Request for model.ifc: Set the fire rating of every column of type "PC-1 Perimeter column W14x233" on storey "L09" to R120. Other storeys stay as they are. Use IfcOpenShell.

First a look at what the model holds.

```python
import ifcopenshell
import ifcopenshell.util.element

model = ifcopenshell.open("model.ifc")
print(model.schema)
storey = next(s for s in model.by_type("IfcBuildingStorey") if s.Name == "L09")
columns = [e for e in ifcopenshell.util.element.get_decomposition(storey) if e.is_a("IfcColumn")]
seen = {}
for e in columns:
    element_type = ifcopenshell.util.element.get_type(e)
    key = (element_type.Name if element_type != e and element_type else None, ifcopenshell.util.element.get_pset(e, "Pset_ColumnCommon", "FireRating"))
    seen[key] = seen.get(key, 0) + 1
for (name, value), count in sorted(seen.items(), key=str):
    print(count, "x", name, "|", value)
```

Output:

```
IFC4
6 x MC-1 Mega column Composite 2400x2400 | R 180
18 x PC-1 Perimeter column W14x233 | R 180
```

```python
import ifcopenshell
import ifcopenshell.api.pset
import ifcopenshell.util.element

model = ifcopenshell.open("model.ifc")

storey = next(s for s in model.by_type("IfcBuildingStorey") if s.Name == "L09")
columns = [e for e in ifcopenshell.util.element.get_decomposition(storey) if e.is_a("IfcColumn")]

count = 0
for e in columns:
    element_type = ifcopenshell.util.element.get_type(e)
    if element_type in (None, e) or element_type.Name != "PC-1 Perimeter column W14x233":
        continue
    found = ifcopenshell.util.element.get_pset(e, "Pset_ColumnCommon", should_inherit=False)
    if found:
        pset = model.by_id(found["id"])
        if len(ifcopenshell.util.element.get_elements_by_pset(pset)) > 1:
            pset = ifcopenshell.api.pset.unshare_pset(model, products=[e], pset=pset)[0]
    else:
        pset = ifcopenshell.api.pset.add_pset(model, product=e, name="Pset_ColumnCommon")
    ifcopenshell.api.pset.edit_pset(model, pset=pset, properties={"FireRating": "R120"})
    count += 1

print(count, "columns updated")

model.write("model-out.ifc")
```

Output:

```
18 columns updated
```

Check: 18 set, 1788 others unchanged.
